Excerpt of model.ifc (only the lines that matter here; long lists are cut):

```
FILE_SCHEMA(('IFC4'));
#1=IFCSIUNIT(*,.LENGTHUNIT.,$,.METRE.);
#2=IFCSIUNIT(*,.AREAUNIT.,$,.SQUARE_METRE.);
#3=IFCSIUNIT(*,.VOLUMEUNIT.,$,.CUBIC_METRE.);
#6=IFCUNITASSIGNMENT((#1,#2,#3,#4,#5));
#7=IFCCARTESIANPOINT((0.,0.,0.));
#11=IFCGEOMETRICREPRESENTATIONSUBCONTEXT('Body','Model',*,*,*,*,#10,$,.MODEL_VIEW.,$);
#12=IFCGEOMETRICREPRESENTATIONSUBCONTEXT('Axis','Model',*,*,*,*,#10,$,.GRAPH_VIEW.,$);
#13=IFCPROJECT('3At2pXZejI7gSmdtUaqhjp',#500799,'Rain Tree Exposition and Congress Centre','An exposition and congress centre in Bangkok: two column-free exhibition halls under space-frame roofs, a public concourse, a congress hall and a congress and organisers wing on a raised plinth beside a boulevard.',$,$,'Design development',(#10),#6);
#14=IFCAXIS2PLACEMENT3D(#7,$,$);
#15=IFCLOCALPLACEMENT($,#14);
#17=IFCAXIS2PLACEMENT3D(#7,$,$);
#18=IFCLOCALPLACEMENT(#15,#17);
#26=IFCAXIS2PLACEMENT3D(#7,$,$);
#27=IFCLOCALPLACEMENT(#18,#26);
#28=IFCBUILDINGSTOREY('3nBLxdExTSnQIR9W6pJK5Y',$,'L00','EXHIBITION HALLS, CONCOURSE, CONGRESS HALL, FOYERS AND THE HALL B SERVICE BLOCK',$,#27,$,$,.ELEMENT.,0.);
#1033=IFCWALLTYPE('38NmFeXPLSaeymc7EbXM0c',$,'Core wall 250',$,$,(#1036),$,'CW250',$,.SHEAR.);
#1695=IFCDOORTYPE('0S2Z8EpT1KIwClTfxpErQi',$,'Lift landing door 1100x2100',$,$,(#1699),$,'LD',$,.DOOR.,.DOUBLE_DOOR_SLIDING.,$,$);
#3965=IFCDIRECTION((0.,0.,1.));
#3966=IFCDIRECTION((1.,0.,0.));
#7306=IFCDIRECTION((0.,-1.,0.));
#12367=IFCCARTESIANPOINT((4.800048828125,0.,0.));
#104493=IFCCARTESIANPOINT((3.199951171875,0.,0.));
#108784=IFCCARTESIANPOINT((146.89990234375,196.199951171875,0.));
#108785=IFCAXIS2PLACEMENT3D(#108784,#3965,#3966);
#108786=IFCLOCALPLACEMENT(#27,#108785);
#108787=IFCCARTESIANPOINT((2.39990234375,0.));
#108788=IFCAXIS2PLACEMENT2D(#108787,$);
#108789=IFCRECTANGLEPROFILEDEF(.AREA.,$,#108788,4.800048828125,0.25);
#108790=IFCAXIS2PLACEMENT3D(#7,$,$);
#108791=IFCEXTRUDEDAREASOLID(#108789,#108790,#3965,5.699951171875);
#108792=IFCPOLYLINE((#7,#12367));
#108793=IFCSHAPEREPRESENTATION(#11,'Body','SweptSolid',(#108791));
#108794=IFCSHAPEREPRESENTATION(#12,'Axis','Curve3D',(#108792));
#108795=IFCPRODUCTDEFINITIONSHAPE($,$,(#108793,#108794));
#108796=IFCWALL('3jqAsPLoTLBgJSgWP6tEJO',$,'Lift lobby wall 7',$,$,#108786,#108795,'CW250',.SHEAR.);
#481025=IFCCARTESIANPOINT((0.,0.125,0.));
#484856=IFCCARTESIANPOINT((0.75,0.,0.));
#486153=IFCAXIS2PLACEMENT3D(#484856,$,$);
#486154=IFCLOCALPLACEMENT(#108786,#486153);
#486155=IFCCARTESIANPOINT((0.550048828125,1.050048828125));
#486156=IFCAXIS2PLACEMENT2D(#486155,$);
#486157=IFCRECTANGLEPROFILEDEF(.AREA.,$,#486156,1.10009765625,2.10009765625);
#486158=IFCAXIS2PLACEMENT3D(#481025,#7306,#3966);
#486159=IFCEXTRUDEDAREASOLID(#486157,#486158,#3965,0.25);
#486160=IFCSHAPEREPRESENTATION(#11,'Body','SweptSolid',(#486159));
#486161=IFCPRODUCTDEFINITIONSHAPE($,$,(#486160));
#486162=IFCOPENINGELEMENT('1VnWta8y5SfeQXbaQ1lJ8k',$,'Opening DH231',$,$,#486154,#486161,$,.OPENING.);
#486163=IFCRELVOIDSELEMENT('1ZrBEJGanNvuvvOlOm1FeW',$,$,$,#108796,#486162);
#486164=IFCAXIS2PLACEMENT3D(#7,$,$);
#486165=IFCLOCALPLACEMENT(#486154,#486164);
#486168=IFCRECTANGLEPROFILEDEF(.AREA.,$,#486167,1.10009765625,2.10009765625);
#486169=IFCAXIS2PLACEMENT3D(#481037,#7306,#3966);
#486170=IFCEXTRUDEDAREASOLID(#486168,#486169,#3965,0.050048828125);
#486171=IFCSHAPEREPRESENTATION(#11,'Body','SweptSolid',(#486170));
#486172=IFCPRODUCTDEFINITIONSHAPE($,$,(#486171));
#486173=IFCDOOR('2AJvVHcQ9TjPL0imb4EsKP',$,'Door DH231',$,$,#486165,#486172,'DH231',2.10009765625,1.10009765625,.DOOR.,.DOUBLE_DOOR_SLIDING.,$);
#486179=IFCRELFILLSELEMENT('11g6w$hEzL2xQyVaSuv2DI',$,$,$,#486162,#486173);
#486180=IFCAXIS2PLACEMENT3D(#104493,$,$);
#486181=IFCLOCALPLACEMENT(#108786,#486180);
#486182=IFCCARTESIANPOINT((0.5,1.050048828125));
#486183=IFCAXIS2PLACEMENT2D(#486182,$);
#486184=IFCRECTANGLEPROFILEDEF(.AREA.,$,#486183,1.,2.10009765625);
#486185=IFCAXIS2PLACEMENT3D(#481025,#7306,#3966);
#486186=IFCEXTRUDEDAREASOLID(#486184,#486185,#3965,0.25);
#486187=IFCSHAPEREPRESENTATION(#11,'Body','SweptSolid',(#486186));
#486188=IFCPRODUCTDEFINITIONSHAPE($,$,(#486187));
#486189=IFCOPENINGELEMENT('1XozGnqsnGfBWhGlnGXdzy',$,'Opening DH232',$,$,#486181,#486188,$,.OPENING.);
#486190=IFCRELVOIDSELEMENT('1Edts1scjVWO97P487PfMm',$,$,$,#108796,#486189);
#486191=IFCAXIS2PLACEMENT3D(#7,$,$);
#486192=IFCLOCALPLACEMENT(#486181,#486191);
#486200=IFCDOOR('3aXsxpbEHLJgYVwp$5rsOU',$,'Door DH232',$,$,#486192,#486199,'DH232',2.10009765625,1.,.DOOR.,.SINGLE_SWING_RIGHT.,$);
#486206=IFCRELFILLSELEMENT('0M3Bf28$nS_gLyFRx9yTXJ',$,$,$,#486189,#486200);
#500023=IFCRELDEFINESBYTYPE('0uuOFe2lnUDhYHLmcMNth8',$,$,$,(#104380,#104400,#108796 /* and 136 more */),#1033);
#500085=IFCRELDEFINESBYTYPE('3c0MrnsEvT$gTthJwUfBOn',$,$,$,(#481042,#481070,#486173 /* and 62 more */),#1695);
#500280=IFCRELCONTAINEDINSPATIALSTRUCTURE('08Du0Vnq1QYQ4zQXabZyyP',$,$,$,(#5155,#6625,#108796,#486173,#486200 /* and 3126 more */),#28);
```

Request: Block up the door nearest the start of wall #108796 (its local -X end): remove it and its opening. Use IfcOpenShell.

```python
import ifcopenshell
import ifcopenshell.api.feature
import ifcopenshell.api.root
import ifcopenshell.geom
import ifcopenshell.util.shape

model = ifcopenshell.open("model.ifc")
settings = ifcopenshell.geom.settings()


def volume(element):
    """Net volume in cubic metres, openings subtracted."""
    shape = ifcopenshell.geom.create_shape(settings, element)
    return ifcopenshell.util.shape.get_volume(shape.geometry)


door = model.by_guid("2AJvVHcQ9TjPL0imb4EsKP")
opening = door.FillsVoids[0].RelatingOpeningElement
wall = opening.VoidsElements[0].RelatingBuildingElement
before = volume(wall)

ifcopenshell.api.root.remove_product(model, product=door)
ifcopenshell.api.feature.remove_feature(model, feature=opening)

after = volume(wall)

print(f"wall volume {before:.3f} -> {after:.3f} m3")

model.write("model_updated.ifc")
```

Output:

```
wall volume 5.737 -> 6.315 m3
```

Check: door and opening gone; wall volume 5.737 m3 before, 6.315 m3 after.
